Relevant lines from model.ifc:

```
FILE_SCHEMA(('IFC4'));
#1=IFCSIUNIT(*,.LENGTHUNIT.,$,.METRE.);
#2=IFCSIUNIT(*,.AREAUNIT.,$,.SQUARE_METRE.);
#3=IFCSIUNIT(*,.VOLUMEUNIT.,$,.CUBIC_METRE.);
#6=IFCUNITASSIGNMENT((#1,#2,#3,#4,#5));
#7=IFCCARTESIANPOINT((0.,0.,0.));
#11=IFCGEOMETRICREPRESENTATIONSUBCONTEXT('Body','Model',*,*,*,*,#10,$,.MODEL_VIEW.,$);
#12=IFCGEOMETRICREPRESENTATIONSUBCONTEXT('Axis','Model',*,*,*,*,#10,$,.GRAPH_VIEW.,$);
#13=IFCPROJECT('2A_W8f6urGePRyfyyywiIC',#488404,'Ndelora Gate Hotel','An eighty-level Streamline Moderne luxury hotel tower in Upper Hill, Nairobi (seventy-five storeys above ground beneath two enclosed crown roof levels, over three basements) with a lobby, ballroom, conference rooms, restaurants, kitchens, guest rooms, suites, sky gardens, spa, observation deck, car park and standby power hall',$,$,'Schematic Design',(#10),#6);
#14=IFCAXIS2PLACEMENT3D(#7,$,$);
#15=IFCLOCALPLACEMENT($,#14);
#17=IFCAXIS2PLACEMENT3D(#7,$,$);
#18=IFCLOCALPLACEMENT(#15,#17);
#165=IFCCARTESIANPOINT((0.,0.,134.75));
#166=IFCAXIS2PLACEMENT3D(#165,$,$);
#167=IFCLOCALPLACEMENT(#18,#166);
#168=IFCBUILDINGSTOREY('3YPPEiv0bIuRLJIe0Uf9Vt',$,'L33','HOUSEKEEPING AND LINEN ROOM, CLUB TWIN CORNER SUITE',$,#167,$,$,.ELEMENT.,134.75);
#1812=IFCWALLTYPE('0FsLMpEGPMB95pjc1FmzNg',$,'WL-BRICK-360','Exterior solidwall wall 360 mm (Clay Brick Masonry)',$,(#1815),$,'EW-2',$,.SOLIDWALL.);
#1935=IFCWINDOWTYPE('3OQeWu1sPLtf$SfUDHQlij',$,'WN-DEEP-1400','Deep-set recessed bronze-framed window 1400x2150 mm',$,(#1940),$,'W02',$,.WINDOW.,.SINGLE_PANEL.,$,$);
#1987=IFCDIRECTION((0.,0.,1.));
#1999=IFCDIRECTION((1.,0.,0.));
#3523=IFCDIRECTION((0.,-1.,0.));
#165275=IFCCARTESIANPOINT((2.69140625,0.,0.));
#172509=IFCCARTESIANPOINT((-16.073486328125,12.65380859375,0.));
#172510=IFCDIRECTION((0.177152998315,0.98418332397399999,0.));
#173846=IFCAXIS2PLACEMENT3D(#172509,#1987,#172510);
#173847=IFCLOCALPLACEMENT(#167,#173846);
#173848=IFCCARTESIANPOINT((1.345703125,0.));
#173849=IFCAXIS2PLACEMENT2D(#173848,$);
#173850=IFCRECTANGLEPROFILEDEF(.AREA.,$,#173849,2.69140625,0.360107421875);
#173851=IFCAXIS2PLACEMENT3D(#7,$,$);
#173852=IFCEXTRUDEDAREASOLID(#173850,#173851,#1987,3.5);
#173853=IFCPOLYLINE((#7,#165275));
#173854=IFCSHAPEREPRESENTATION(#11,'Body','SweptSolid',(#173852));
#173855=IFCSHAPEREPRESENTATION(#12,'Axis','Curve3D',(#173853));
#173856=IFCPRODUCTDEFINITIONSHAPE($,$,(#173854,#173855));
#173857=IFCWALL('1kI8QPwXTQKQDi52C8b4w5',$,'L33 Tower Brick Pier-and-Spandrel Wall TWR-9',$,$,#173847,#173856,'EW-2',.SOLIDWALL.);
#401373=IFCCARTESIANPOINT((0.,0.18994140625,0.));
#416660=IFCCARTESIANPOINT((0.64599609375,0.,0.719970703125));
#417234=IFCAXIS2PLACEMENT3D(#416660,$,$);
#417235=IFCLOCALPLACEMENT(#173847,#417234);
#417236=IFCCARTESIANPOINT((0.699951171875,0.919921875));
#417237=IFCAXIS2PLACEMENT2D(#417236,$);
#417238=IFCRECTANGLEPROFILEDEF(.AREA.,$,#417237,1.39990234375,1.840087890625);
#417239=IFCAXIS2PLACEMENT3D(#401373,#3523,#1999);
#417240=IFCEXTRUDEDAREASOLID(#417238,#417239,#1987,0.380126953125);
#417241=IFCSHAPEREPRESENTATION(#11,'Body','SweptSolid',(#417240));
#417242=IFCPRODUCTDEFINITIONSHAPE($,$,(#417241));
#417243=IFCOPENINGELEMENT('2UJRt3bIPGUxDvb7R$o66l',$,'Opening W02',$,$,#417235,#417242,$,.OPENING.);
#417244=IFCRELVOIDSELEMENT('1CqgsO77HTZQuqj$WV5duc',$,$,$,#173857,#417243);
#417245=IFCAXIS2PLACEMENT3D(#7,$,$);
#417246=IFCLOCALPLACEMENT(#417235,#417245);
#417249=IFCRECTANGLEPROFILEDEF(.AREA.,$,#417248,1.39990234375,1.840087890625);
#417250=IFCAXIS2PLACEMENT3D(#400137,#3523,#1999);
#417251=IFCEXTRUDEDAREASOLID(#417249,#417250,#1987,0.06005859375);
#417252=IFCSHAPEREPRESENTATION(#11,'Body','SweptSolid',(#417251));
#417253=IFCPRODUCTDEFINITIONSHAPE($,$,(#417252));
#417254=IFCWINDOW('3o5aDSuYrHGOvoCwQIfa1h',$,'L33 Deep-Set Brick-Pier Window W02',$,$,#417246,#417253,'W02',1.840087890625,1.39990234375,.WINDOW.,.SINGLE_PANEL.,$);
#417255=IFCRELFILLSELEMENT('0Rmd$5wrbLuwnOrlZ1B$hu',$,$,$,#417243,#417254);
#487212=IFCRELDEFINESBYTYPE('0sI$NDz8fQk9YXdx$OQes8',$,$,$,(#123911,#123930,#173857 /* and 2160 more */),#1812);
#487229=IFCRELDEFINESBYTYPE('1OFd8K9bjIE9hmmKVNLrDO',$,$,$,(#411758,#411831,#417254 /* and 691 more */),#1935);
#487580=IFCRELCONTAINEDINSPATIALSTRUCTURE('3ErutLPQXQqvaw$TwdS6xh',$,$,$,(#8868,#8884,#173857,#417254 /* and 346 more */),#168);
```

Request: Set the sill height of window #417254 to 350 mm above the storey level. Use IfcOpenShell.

```python
import numpy as np
import ifcopenshell
import ifcopenshell.api.geometry
import ifcopenshell.geom
import ifcopenshell.util.element
import ifcopenshell.util.placement
import ifcopenshell.util.shape
import ifcopenshell.util.unit

model = ifcopenshell.open("model.ifc")
unit_scale = ifcopenshell.util.unit.calculate_unit_scale(model)

window = model.by_guid("3o5aDSuYrHGOvoCwQIfa1h")
opening = window.FillsVoids[0].RelatingOpeningElement
storey = ifcopenshell.util.element.get_container(window, ifc_class="IfcBuildingStorey")
level = ifcopenshell.util.placement.get_local_placement(storey.ObjectPlacement)[2, 3]

# The opening's origin need not be at the sill, so measure its lowest point.
shape = ifcopenshell.geom.create_shape(ifcopenshell.geom.settings(), opening)
bottom = ifcopenshell.util.shape.get_shape_bottom_elevation(shape, shape.geometry) / unit_scale
dz = level + 0.35 / unit_scale - bottom

shift = np.array([0.0, 0.0, dz])
# The window is placed relative to its opening, so it follows when the opening moves.
matrix = ifcopenshell.util.placement.get_local_placement(opening.ObjectPlacement)
matrix[:3, 3] += shift
ifcopenshell.api.geometry.edit_object_placement(
    model, product=opening, matrix=matrix, is_si=False, should_transform_children=True
)

print(f"moved by {dz * unit_scale:+.3f} m")

model.write("model_v2.ifc")
```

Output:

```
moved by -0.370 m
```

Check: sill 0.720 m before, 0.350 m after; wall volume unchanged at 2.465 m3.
